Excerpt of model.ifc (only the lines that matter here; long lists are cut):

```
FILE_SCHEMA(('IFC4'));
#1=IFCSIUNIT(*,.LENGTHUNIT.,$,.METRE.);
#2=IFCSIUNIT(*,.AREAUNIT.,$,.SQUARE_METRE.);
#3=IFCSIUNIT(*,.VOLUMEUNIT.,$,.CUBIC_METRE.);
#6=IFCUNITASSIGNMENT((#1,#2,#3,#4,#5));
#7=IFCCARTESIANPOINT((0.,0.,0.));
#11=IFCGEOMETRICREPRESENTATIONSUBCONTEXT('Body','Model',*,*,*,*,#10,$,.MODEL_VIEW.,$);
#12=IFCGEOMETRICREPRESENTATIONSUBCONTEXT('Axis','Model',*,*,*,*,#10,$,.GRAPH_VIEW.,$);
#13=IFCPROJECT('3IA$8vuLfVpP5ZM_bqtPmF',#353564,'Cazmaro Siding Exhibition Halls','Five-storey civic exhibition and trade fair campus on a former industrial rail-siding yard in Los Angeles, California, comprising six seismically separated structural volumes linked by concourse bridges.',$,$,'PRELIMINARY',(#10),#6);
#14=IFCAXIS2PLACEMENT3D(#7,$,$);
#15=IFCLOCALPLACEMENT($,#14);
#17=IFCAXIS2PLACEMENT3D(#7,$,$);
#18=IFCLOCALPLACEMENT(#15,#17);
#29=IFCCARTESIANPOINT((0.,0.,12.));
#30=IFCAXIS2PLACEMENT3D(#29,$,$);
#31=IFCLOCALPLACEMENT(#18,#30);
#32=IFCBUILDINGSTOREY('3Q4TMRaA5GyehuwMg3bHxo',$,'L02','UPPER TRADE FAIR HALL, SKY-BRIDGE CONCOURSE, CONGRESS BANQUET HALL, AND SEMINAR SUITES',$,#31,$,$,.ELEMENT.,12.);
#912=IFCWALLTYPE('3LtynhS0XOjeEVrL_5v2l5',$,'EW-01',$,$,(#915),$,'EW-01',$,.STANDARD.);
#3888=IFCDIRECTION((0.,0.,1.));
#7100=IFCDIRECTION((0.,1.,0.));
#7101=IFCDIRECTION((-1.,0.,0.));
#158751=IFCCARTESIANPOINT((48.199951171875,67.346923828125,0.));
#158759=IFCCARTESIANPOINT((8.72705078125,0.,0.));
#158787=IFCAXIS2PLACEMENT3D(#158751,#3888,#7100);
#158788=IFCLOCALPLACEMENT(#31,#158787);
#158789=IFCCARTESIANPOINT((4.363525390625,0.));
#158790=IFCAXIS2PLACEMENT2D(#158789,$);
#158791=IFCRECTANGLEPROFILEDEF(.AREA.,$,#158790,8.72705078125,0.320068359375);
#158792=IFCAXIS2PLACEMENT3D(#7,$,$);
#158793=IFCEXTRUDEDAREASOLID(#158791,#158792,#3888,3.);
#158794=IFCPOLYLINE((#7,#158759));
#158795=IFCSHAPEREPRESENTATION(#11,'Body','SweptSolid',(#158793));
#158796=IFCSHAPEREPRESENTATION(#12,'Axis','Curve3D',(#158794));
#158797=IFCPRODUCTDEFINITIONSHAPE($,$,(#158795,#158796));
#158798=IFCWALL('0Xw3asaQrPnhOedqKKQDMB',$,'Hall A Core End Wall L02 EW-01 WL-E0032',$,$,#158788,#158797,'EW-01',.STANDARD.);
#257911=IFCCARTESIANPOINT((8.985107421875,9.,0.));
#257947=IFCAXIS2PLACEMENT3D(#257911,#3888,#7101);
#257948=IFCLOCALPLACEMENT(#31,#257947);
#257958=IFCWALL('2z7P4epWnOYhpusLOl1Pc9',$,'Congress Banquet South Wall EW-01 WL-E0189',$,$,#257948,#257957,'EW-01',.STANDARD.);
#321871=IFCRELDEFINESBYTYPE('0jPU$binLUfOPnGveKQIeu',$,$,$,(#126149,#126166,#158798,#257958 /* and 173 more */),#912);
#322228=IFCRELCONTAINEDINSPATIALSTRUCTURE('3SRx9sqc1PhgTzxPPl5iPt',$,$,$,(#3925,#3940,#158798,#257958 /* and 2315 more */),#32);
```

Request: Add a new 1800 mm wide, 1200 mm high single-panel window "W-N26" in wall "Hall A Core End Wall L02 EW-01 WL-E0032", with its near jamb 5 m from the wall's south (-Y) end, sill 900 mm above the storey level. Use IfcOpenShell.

```python
import numpy as np
import ifcopenshell
import ifcopenshell.api.feature
import ifcopenshell.api.geometry
import ifcopenshell.api.root
import ifcopenshell.api.spatial
import ifcopenshell.geom
import ifcopenshell.util.element
import ifcopenshell.util.placement
import ifcopenshell.util.representation
import ifcopenshell.util.shape
import ifcopenshell.util.unit

model = ifcopenshell.open("model.ifc")
unit_scale = ifcopenshell.util.unit.calculate_unit_scale(model)
settings = ifcopenshell.geom.settings()


def volume(element):
    """Net volume in cubic metres, openings subtracted."""
    shape = ifcopenshell.geom.create_shape(settings, element)
    return ifcopenshell.util.shape.get_volume(shape.geometry)


wall = model.by_id(158798)
storey = ifcopenshell.util.element.get_container(wall, ifc_class="IfcBuildingStorey")
context = ifcopenshell.util.representation.get_context(model, "Model", "Body", "MODEL_VIEW")
before = volume(wall)

width, height, from_end, sill = 1.8, 1.2, 5, 0.9  # metres

# The wall runs along its own X axis, and the end named is its -X end.
wall_shape = ifcopenshell.geom.create_shape(settings, wall)
x, y, z = ifcopenshell.util.shape.get_vertices(wall_shape.geometry).T
start = x.min() + from_end
face, thickness = float(y.min()), float(y.max() - y.min())
wall_matrix = ifcopenshell.util.placement.get_local_placement(wall.ObjectPlacement)
level = ifcopenshell.util.placement.get_local_placement(storey.ObjectPlacement)[2, 3]


def in_wall(x, y):
    """Placement at x, y metres in the wall's axes, at sill height."""
    matrix = wall_matrix.copy()
    matrix[:, 3] = wall_matrix @ np.array([x / unit_scale, y / unit_scale, 0.0, 1.0])
    matrix[2, 3] = level + sill / unit_scale
    return matrix


# Opening: a box that overshoots both wall faces by 50 mm.
opening = ifcopenshell.api.root.create_entity(model, ifc_class="IfcOpeningElement", predefined_type="OPENING")
box = ifcopenshell.api.geometry.add_wall_representation(
    model, context=context, length=width, height=height, thickness=thickness + 0.1
)
ifcopenshell.api.geometry.assign_representation(model, product=opening, representation=box)
ifcopenshell.api.geometry.edit_object_placement(model, product=opening, matrix=in_wall(start, face - 0.05), is_si=False)
ifcopenshell.api.feature.add_feature(model, feature=opening, element=wall)

window = ifcopenshell.api.root.create_entity(model, ifc_class="IfcWindow", name="W-N26", predefined_type="WINDOW")
window.OverallWidth, window.OverallHeight = width / unit_scale, height / unit_scale
window.PartitioningType = "SINGLE_PANEL"
body = ifcopenshell.api.geometry.add_window_representation(
    model,
    context=context,
    overall_width=window.OverallWidth,
    overall_height=window.OverallHeight,
    partition_type="SINGLE_PANEL",
)
ifcopenshell.api.geometry.assign_representation(model, product=window, representation=body)
ifcopenshell.api.spatial.assign_container(model, products=[window], relating_structure=storey)
ifcopenshell.api.feature.add_filling(model, opening=opening, element=window)

# Centre the window in the wall's thickness.
ifcopenshell.api.geometry.edit_object_placement(model, product=window, matrix=in_wall(start, face), is_si=False)
window_shape = ifcopenshell.geom.create_shape(settings, window)
depth = ifcopenshell.util.shape.get_vertices(window_shape.geometry)[:, 1]
offset = face + thickness / 2 - (depth.min() + depth.max()) / 2
ifcopenshell.api.geometry.edit_object_placement(model, product=window, matrix=in_wall(start, offset), is_si=False)

after = volume(wall)

print(f"wall volume {before:.3f} -> {after:.3f} m3")

model.write("model-out.ifc")
```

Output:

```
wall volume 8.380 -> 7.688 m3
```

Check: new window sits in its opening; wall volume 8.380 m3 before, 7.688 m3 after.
